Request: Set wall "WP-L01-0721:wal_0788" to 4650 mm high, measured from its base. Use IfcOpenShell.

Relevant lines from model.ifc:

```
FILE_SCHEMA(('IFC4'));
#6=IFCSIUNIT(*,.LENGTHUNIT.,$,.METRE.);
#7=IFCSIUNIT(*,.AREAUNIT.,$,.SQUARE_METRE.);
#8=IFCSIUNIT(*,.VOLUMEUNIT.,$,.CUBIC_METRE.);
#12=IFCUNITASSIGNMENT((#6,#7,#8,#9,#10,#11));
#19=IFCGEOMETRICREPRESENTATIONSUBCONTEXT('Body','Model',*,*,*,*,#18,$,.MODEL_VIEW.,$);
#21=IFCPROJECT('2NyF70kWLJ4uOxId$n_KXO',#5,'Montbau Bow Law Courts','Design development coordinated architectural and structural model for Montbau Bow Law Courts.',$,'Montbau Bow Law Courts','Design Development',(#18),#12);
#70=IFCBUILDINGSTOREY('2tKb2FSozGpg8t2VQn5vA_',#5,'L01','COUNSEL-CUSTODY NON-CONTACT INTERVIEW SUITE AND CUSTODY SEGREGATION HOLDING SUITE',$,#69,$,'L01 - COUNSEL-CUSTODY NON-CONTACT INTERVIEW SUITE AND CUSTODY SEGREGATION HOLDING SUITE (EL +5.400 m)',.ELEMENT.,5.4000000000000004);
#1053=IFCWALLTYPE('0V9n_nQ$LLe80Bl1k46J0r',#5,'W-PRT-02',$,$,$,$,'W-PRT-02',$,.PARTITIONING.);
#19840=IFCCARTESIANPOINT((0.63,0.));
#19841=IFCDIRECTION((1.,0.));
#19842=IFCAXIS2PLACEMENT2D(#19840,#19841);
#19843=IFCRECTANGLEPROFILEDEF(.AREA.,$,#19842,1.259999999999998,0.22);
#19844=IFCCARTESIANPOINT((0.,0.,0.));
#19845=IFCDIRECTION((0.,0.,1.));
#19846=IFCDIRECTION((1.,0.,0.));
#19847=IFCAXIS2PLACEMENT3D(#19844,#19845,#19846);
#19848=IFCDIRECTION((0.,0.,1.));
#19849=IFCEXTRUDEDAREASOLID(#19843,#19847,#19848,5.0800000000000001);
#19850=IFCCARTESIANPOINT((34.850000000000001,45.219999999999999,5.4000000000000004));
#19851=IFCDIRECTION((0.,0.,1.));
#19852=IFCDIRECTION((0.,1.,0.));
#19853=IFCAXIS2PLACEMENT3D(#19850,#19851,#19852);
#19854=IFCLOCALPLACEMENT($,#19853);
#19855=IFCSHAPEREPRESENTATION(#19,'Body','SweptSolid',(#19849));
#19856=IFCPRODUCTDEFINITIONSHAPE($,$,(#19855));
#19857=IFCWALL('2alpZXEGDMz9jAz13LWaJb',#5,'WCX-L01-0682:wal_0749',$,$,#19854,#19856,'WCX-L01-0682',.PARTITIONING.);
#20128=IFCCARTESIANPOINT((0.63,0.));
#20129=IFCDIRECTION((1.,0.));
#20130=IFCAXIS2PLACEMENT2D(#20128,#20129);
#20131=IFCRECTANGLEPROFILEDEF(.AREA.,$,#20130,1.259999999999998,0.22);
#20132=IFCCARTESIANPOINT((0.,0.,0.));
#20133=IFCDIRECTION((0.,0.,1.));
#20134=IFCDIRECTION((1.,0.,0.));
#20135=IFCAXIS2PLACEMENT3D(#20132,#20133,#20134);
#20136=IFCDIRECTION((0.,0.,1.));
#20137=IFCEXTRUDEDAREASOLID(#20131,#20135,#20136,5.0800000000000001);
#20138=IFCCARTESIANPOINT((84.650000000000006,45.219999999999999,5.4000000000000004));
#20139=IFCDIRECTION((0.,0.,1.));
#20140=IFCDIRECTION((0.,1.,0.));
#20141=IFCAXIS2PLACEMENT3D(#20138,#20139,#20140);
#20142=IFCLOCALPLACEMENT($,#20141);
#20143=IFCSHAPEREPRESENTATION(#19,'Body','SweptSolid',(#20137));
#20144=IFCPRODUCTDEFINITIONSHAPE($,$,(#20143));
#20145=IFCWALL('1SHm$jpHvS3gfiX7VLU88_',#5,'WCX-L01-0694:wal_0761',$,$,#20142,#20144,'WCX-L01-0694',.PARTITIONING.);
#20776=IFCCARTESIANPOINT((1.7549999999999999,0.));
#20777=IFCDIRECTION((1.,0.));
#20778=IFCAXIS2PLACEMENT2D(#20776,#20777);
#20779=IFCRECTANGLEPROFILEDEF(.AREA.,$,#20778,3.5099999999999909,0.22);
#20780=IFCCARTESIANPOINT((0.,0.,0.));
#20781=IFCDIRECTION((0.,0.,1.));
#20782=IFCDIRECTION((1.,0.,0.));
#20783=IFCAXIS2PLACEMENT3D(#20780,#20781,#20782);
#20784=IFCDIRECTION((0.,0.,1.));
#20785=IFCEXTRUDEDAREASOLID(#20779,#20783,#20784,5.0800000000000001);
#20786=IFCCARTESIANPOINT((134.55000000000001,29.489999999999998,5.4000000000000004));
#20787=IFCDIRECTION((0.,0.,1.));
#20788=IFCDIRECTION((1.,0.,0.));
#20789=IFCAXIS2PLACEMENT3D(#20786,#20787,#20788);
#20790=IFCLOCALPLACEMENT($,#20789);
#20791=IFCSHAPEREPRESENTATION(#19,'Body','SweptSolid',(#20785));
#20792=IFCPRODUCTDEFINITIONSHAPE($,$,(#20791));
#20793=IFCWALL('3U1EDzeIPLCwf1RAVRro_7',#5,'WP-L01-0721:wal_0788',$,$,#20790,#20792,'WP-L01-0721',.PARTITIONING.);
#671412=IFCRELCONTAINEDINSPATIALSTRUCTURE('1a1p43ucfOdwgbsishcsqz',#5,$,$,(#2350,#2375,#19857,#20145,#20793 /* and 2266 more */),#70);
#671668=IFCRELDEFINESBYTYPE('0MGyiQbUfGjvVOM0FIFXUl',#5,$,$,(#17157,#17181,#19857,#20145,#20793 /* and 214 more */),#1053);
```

```python
import ifcopenshell
import ifcopenshell.geom
import ifcopenshell.util.representation
import ifcopenshell.util.shape
import ifcopenshell.util.unit

model = ifcopenshell.open("model.ifc")
unit_scale = ifcopenshell.util.unit.calculate_unit_scale(model)
settings = ifcopenshell.geom.settings()


def volume(element):
    """Net volume in cubic metres, openings subtracted."""
    shape = ifcopenshell.geom.create_shape(settings, element)
    return ifcopenshell.util.shape.get_volume(shape.geometry)


wall = model.by_id(20793)
before = volume(wall)

body = ifcopenshell.util.representation.get_representation(wall, "Model", "Body")
solid = body.Items[0]
old_height = solid.Depth
solid.Depth = 4.65 / unit_scale
after = volume(wall)

print(f"height {old_height:g} -> {solid.Depth:g}, volume {before:.3f} -> {after:.3f} m3")

model.write("model_v2.ifc")
```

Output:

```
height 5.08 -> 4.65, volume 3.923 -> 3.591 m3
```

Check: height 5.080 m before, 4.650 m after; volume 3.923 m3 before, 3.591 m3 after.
